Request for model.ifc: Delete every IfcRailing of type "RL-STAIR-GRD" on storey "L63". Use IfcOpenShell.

First a look at what the model holds.

```python
import ifcopenshell
import ifcopenshell.util.element

model = ifcopenshell.open("model.ifc")
print(model.schema)
storey = next(s for s in model.by_type("IfcBuildingStorey") if s.Name == "L63")
railings = [e for e in ifcopenshell.util.element.get_decomposition(storey) if e.is_a("IfcRailing")]
seen = {}
for e in railings:
    element_type = ifcopenshell.util.element.get_type(e)
    name = element_type.Name if element_type not in (None, e) else None
    seen[name] = seen.get(name, 0) + 1
for name, count in sorted(seen.items(), key=str):
    print(count, "x", name)
```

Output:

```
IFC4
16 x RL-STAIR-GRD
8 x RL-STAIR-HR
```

```python
import ifcopenshell
import ifcopenshell.api.root
import ifcopenshell.util.element

model = ifcopenshell.open("model.ifc")

storey = next(s for s in model.by_type("IfcBuildingStorey") if s.Name == "L63")
railings = [e for e in ifcopenshell.util.element.get_decomposition(storey) if e.is_a("IfcRailing")]
targets = [e for e in railings if (t := ifcopenshell.util.element.get_type(e)) not in (None, e) and t.Name == "RL-STAIR-GRD"]

for e in targets:
    ifcopenshell.api.root.remove_product(model, product=e)
print(len(targets), "removed")

model.write("model_updated.ifc")
```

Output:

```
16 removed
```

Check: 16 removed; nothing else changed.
